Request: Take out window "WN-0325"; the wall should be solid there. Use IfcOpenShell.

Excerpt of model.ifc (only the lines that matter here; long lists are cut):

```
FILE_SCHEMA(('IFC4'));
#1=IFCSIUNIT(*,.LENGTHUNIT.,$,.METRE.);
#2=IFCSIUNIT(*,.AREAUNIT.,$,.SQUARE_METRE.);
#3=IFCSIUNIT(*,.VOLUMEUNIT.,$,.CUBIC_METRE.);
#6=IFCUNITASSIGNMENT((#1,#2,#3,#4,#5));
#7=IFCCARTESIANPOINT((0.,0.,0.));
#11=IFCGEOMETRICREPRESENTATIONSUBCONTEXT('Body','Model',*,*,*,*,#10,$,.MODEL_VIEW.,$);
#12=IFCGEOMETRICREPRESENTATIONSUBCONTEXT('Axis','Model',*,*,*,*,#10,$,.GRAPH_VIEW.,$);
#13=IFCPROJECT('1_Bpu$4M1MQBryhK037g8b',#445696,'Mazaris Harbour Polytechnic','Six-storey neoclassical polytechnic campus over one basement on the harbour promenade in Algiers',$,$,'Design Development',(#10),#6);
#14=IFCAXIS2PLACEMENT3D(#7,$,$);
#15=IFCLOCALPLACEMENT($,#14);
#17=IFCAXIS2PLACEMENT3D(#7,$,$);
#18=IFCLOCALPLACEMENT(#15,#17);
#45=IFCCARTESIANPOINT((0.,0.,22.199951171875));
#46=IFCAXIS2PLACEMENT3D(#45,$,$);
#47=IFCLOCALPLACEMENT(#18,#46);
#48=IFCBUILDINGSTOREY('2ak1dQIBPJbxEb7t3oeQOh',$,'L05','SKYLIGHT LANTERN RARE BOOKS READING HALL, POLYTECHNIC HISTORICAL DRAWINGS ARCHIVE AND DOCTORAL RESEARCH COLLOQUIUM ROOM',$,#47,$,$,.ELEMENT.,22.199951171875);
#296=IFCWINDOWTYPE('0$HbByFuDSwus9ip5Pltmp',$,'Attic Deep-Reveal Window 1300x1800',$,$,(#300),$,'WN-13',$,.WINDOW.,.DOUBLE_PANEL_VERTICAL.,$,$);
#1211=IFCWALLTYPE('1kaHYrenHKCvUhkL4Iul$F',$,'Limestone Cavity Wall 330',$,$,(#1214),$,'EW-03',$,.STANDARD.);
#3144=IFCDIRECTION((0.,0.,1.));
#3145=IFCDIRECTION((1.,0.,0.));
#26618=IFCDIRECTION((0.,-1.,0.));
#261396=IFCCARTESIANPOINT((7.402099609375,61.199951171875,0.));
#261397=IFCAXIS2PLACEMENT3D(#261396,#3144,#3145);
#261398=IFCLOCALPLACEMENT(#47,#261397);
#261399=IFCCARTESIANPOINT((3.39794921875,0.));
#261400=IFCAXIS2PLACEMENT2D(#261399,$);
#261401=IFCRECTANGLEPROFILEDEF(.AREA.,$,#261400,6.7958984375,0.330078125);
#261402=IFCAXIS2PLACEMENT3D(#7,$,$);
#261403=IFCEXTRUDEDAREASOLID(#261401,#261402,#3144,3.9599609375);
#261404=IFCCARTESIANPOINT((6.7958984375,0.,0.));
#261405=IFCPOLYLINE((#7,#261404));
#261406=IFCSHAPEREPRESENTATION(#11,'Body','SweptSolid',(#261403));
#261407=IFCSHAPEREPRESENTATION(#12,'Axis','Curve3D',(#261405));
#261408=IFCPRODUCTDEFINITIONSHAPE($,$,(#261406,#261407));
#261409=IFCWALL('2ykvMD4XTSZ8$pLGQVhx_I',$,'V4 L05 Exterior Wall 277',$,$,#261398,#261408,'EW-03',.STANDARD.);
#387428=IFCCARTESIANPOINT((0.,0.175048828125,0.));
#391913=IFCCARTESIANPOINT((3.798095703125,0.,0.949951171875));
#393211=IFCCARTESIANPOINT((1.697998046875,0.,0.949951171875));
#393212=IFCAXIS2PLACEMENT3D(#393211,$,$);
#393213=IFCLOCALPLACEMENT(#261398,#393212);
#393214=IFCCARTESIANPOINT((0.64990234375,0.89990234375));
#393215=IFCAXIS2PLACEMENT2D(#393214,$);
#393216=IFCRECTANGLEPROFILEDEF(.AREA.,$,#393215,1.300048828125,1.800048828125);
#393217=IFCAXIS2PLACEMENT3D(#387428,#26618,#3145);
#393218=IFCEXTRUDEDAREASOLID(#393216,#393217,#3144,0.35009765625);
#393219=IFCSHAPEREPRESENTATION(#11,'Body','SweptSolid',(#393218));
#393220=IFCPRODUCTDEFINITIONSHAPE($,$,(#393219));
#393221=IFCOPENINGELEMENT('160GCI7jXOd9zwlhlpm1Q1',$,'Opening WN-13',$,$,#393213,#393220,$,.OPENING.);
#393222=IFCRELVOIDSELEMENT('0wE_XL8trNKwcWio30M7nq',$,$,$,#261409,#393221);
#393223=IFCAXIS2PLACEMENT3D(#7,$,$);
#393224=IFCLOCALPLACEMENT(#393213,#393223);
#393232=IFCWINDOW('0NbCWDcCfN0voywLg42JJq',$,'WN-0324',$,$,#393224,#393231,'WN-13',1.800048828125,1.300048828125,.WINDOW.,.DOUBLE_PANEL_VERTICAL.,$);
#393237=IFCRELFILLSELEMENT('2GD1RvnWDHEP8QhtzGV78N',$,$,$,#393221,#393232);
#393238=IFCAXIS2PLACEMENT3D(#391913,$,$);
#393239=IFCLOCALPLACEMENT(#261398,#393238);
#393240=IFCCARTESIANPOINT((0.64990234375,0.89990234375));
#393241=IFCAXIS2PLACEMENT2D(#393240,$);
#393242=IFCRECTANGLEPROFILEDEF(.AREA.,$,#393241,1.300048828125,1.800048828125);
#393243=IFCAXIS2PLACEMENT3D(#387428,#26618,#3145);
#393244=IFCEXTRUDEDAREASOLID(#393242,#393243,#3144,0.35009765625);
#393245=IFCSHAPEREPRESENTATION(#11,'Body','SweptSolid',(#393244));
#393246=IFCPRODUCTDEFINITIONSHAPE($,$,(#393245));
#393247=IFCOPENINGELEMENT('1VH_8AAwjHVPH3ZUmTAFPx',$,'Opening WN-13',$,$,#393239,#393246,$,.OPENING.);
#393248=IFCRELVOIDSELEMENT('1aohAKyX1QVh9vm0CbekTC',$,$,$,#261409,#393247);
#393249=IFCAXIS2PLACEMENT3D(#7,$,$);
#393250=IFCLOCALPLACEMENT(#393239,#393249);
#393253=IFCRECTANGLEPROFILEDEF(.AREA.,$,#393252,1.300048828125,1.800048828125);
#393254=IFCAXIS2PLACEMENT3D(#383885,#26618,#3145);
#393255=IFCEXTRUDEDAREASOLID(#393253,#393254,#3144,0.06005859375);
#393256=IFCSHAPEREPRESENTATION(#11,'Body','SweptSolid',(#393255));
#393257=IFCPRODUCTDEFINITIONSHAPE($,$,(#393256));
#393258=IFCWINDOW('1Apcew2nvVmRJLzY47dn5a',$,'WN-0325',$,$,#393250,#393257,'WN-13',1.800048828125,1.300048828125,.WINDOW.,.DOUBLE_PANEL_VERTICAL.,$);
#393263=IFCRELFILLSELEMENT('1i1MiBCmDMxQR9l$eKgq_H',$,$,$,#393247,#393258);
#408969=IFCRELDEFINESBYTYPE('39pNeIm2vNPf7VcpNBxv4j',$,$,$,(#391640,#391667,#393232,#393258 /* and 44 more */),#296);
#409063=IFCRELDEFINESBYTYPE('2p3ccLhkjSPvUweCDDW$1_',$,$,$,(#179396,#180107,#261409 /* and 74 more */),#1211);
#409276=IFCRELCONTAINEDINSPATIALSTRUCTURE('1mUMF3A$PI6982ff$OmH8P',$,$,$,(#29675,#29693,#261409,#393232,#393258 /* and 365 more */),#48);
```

```python
import ifcopenshell
import ifcopenshell.api.feature
import ifcopenshell.api.root
import ifcopenshell.geom
import ifcopenshell.util.shape

model = ifcopenshell.open("model.ifc")
settings = ifcopenshell.geom.settings()


def volume(element):
    """Net volume in cubic metres, openings subtracted."""
    shape = ifcopenshell.geom.create_shape(settings, element)
    return ifcopenshell.util.shape.get_volume(shape.geometry)


window = model.by_id(393258)
opening = window.FillsVoids[0].RelatingOpeningElement
wall = opening.VoidsElements[0].RelatingBuildingElement
before = volume(wall)

ifcopenshell.api.root.remove_product(model, product=window)
ifcopenshell.api.feature.remove_feature(model, feature=opening)

after = volume(wall)

print(f"wall volume {before:.3f} -> {after:.3f} m3")

model.write("model_edited.ifc")
```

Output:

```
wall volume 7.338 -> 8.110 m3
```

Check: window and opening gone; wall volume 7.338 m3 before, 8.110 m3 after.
